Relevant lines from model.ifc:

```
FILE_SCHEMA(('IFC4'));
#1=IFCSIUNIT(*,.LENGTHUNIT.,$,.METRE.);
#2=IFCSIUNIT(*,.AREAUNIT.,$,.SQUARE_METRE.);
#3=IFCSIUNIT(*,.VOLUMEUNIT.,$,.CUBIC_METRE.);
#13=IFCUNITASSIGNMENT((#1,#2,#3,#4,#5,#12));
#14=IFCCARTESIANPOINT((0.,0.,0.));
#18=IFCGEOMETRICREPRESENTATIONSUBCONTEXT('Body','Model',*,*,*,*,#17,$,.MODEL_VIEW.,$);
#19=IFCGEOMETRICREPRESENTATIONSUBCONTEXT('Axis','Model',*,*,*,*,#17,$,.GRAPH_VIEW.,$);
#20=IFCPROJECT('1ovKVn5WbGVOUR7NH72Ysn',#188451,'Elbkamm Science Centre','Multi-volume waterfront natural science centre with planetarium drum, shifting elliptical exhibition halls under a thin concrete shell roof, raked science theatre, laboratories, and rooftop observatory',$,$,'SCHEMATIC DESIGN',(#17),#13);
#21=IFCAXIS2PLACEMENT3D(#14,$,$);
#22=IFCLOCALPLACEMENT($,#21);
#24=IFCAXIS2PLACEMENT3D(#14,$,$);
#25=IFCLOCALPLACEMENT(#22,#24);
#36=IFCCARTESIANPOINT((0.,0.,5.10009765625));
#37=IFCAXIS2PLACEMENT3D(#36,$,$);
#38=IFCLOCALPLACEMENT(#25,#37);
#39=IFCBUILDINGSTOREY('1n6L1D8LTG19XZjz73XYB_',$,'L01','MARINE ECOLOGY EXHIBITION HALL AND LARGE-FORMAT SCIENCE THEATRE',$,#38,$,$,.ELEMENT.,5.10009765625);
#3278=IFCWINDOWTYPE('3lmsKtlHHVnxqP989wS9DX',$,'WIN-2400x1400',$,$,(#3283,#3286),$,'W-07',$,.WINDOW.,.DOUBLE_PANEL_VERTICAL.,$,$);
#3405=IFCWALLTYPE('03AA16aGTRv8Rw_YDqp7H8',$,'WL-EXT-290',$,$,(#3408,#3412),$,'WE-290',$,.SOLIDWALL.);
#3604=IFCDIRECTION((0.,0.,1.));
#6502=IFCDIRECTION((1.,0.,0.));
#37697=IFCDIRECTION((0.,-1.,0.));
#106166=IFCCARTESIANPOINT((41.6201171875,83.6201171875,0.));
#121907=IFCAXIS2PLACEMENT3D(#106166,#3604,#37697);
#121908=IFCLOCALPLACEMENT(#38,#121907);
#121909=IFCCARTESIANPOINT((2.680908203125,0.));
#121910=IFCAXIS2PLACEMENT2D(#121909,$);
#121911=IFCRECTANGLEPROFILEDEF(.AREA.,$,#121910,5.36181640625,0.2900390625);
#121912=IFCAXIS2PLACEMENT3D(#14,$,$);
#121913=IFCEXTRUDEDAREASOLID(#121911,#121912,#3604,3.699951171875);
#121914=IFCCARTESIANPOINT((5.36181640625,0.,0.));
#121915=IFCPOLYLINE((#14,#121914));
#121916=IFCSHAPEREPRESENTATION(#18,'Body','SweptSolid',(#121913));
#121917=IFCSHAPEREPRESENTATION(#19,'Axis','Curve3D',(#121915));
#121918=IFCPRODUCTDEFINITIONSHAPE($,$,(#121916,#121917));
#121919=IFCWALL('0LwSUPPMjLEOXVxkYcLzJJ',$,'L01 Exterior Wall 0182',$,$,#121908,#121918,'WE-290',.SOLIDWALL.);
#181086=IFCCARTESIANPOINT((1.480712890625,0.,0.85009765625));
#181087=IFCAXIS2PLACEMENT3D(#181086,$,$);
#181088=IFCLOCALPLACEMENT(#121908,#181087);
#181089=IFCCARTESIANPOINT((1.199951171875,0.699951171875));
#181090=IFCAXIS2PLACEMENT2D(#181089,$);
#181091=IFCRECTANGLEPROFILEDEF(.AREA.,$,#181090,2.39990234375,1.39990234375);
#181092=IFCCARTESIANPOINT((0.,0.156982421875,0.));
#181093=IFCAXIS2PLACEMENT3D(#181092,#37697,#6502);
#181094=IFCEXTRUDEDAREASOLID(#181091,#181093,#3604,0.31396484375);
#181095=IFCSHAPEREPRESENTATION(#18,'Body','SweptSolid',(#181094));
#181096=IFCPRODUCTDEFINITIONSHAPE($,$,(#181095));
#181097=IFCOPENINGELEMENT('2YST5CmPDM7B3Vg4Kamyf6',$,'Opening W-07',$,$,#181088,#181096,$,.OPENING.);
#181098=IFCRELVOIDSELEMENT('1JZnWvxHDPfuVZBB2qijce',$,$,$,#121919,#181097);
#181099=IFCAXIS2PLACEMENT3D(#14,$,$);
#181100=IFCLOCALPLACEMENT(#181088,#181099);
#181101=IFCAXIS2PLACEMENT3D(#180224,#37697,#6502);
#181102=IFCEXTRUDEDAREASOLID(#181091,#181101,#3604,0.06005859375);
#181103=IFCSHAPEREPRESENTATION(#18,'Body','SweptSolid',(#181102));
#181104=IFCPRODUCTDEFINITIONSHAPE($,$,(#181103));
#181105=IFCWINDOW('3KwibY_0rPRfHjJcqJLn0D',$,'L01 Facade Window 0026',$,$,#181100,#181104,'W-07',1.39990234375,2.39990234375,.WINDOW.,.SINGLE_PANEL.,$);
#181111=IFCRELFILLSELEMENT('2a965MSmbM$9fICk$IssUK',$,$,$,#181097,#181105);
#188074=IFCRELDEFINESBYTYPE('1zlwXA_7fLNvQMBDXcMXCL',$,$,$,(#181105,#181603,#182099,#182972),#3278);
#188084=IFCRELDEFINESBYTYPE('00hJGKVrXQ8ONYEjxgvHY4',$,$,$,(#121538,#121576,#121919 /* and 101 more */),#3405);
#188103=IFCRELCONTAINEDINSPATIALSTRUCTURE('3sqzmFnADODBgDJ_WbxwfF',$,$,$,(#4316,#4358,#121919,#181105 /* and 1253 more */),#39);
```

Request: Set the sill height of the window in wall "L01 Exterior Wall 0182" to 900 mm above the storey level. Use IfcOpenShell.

```python
import numpy as np
import ifcopenshell
import ifcopenshell.api.geometry
import ifcopenshell.geom
import ifcopenshell.util.element
import ifcopenshell.util.placement
import ifcopenshell.util.shape
import ifcopenshell.util.unit

model = ifcopenshell.open("model.ifc")
unit_scale = ifcopenshell.util.unit.calculate_unit_scale(model)

window = model.by_id(181105)
opening = window.FillsVoids[0].RelatingOpeningElement
storey = ifcopenshell.util.element.get_container(window, ifc_class="IfcBuildingStorey")
level = ifcopenshell.util.placement.get_local_placement(storey.ObjectPlacement)[2, 3]

# The opening's origin need not be at the sill, so measure its lowest point.
shape = ifcopenshell.geom.create_shape(ifcopenshell.geom.settings(), opening)
bottom = ifcopenshell.util.shape.get_shape_bottom_elevation(shape, shape.geometry) / unit_scale
dz = level + 0.9 / unit_scale - bottom

shift = np.array([0.0, 0.0, dz])
# The window is placed relative to its opening, so it follows when the opening moves.
matrix = ifcopenshell.util.placement.get_local_placement(opening.ObjectPlacement)
matrix[:3, 3] += shift
ifcopenshell.api.geometry.edit_object_placement(
    model, product=opening, matrix=matrix, is_si=False, should_transform_children=True
)

print(f"moved by {dz * unit_scale:+.3f} m")

model.write("model_updated.ifc")
```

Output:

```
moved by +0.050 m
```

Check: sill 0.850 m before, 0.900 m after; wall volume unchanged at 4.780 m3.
